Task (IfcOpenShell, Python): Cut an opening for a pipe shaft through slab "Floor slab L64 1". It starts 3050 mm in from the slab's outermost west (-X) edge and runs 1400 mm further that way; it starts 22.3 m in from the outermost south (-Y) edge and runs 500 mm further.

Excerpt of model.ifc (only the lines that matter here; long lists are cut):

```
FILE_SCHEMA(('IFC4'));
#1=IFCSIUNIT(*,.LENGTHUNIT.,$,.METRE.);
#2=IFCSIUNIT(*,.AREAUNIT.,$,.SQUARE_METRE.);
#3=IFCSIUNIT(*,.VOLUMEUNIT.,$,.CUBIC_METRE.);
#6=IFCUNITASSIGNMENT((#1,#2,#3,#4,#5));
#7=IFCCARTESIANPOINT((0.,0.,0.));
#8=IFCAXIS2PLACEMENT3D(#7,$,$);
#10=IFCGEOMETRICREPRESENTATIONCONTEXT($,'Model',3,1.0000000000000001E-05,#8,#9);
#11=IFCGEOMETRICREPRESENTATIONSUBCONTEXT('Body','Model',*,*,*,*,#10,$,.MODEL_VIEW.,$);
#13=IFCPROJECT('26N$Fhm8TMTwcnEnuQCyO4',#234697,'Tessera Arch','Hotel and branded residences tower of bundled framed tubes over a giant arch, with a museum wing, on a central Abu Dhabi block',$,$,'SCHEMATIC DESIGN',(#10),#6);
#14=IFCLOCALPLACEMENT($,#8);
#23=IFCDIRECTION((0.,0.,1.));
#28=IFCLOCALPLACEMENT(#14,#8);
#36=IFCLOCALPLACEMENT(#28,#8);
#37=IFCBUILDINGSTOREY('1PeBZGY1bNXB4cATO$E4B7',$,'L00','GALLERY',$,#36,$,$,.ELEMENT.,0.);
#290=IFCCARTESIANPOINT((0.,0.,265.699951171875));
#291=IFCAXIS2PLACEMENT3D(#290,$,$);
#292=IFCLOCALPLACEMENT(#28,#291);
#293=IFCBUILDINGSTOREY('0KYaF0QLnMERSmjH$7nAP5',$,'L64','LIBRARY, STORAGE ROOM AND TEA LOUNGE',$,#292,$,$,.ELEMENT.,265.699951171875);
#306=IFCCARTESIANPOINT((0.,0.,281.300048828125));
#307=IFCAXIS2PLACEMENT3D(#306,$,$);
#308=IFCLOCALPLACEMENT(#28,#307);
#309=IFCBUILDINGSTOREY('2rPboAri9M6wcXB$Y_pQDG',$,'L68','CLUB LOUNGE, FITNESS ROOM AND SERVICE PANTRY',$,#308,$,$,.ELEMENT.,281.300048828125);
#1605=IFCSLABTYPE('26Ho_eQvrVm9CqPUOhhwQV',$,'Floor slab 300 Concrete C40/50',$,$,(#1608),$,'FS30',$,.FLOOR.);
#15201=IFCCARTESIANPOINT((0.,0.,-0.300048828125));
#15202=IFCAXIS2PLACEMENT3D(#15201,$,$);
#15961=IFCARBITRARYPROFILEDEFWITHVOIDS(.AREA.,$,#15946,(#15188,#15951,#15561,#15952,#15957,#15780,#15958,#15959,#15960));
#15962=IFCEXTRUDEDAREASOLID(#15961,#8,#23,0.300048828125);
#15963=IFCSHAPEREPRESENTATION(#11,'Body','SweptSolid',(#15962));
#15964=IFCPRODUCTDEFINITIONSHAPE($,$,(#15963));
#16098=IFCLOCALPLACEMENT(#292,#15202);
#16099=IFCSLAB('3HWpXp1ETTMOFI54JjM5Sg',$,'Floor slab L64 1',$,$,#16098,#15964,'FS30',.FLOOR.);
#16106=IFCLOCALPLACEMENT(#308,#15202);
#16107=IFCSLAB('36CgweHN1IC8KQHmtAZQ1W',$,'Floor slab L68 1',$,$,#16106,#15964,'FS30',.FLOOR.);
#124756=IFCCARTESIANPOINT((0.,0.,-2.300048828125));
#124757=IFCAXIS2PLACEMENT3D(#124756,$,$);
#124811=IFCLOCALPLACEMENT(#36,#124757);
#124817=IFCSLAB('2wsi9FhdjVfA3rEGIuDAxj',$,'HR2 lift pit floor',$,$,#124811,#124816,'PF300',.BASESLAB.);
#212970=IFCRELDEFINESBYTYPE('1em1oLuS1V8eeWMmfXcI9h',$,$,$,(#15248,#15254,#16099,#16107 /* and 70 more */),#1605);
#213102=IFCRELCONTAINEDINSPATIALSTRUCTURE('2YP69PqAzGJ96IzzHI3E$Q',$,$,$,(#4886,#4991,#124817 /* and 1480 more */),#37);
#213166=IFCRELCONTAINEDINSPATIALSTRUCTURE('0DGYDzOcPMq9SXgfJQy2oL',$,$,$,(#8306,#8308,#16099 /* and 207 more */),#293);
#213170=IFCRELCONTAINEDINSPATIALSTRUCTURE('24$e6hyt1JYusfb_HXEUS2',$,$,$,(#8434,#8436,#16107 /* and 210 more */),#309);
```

```python
import numpy as np
import ifcopenshell
import ifcopenshell.api.feature
import ifcopenshell.api.geometry
import ifcopenshell.api.root
import ifcopenshell.geom
import ifcopenshell.util.placement
import ifcopenshell.util.representation
import ifcopenshell.util.shape
import ifcopenshell.util.unit

model = ifcopenshell.open("model.ifc")
unit_scale = ifcopenshell.util.unit.calculate_unit_scale(model)
settings = ifcopenshell.geom.settings()


def volume(element):
    """Net volume in cubic metres, openings subtracted."""
    shape = ifcopenshell.geom.create_shape(settings, element)
    return ifcopenshell.util.shape.get_volume(shape.geometry)


slab = model.by_id(16099)
before = volume(slab)

# Extent in the slab's own axes, in metres. The edges named are its -X and -Y sides.
slab_shape = ifcopenshell.geom.create_shape(settings, slab)
vertices = ifcopenshell.util.shape.get_vertices(slab_shape.geometry)
x_min, y_min, bottom = vertices.min(axis=0)
top = vertices[:, 2].max()

opening = ifcopenshell.api.root.create_entity(model, ifc_class="IfcOpeningElement", name="Pipe shaft opening", predefined_type="OPENING")
context = ifcopenshell.util.representation.get_context(model, "Model", "Body", "MODEL_VIEW")
width, depth = 1.4, 0.5
outline = [(0.0, 0.0), (width, 0.0), (width, depth), (0.0, depth), (0.0, 0.0)]
# Overshoot both faces by 50 mm so the cut is clean.
shape = ifcopenshell.api.geometry.add_slab_representation(
    model, context=context, depth=top - bottom + 0.1, polyline=outline
)
ifcopenshell.api.geometry.assign_representation(model, product=opening, representation=shape)

matrix = ifcopenshell.util.placement.get_local_placement(slab.ObjectPlacement)
matrix[:, 3] = matrix @ np.append(np.array([x_min + 3.05, y_min + 22.3, bottom - 0.05]) / unit_scale, 1.0)
ifcopenshell.api.geometry.edit_object_placement(model, product=opening, matrix=matrix, is_si=False)
ifcopenshell.api.feature.add_feature(model, feature=opening, element=slab)

after = volume(slab)

print(f"slab volume {before:.3f} -> {after:.3f} m3")

model.write("model-out.ifc")
```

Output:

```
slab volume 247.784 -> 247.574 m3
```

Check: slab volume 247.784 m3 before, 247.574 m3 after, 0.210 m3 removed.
